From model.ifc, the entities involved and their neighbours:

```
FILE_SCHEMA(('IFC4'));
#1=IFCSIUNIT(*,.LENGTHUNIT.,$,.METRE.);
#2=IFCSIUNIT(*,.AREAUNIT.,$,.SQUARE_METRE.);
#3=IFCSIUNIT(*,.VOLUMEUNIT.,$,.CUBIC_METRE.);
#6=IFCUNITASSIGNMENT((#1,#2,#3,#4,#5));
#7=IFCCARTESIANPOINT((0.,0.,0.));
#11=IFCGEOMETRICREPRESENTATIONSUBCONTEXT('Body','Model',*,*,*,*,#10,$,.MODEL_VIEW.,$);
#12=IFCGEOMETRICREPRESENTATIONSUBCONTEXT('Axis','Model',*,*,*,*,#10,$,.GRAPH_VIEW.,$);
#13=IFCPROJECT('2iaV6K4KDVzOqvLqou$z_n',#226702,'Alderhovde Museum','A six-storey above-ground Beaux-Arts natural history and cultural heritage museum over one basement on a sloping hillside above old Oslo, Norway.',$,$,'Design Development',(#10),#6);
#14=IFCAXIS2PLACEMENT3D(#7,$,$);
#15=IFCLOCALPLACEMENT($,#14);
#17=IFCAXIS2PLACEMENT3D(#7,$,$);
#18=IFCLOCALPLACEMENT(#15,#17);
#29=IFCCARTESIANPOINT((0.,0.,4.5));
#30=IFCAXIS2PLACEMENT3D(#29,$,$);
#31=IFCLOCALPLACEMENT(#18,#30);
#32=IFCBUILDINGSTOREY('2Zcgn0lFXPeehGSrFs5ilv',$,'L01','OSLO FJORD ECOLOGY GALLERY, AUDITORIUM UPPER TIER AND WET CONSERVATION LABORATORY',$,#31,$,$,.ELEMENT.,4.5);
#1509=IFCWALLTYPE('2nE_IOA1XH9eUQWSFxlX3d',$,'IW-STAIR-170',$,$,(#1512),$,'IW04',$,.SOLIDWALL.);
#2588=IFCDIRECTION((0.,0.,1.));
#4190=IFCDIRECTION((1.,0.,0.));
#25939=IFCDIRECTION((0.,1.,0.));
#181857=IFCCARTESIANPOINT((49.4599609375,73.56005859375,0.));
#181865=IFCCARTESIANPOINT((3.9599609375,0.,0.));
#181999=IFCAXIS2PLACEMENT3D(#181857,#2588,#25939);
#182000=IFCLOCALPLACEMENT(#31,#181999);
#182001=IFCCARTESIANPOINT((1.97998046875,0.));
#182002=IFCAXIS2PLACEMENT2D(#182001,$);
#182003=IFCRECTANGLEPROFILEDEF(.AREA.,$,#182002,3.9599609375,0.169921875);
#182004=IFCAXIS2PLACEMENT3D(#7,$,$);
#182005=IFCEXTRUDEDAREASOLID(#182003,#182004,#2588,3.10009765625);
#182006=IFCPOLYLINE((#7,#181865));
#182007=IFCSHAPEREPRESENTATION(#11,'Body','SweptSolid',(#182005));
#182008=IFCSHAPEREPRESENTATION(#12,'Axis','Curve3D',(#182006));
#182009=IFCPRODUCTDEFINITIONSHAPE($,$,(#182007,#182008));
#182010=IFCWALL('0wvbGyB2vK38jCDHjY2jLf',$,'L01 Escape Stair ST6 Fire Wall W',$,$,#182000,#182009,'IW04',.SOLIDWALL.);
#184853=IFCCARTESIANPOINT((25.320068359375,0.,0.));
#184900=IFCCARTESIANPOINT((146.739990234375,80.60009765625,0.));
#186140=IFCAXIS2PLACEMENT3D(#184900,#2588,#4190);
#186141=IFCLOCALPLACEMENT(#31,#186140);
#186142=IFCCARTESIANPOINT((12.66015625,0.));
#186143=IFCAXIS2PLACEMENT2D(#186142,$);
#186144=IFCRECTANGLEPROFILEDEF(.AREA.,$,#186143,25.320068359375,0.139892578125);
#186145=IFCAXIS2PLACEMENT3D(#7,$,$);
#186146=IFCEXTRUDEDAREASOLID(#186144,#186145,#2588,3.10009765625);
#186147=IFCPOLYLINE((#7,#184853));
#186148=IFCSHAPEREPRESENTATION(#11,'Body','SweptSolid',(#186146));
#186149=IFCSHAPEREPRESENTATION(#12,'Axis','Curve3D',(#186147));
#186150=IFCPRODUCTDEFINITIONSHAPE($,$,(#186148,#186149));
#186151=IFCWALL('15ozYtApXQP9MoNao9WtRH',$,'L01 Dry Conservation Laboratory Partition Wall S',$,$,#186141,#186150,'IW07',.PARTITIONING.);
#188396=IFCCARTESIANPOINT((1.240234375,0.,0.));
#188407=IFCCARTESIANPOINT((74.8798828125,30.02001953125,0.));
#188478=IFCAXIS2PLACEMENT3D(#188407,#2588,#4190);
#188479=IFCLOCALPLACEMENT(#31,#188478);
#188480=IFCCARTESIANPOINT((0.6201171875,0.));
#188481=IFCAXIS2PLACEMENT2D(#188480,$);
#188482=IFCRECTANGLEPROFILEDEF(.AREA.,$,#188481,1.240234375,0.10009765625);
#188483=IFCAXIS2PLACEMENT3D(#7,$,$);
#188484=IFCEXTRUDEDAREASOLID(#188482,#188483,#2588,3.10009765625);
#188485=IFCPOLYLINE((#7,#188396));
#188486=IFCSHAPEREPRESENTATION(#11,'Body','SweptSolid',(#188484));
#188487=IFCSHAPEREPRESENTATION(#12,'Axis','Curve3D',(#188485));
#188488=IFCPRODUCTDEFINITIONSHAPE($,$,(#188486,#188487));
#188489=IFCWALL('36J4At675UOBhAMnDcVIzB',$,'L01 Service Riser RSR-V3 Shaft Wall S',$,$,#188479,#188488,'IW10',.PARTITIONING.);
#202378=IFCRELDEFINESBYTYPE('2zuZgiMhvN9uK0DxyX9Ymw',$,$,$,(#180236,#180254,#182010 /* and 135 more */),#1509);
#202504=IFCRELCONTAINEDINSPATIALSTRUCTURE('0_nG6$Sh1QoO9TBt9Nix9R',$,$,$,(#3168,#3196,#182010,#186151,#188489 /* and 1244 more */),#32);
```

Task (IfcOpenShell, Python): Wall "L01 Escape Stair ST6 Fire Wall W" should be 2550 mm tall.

```python
import ifcopenshell
import ifcopenshell.geom
import ifcopenshell.util.representation
import ifcopenshell.util.shape

model = ifcopenshell.open("model.ifc")
settings = ifcopenshell.geom.settings()


def volume(element):
    """Net volume in cubic metres, openings subtracted."""
    shape = ifcopenshell.geom.create_shape(settings, element)
    return ifcopenshell.util.shape.get_volume(shape.geometry)


wall = model.by_id(182010)
before = volume(wall)

body = ifcopenshell.util.representation.get_representation(wall, "Model", "Body")
solid = body.Items[0]
old_height = solid.Depth
solid.Depth = 2.55
after = volume(wall)

print(f"height {old_height:g} -> {solid.Depth:g}, volume {before:.3f} -> {after:.3f} m3")

model.write("model_updated.ifc")
```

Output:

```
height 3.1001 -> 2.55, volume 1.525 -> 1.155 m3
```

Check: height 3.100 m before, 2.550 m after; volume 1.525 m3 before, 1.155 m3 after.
